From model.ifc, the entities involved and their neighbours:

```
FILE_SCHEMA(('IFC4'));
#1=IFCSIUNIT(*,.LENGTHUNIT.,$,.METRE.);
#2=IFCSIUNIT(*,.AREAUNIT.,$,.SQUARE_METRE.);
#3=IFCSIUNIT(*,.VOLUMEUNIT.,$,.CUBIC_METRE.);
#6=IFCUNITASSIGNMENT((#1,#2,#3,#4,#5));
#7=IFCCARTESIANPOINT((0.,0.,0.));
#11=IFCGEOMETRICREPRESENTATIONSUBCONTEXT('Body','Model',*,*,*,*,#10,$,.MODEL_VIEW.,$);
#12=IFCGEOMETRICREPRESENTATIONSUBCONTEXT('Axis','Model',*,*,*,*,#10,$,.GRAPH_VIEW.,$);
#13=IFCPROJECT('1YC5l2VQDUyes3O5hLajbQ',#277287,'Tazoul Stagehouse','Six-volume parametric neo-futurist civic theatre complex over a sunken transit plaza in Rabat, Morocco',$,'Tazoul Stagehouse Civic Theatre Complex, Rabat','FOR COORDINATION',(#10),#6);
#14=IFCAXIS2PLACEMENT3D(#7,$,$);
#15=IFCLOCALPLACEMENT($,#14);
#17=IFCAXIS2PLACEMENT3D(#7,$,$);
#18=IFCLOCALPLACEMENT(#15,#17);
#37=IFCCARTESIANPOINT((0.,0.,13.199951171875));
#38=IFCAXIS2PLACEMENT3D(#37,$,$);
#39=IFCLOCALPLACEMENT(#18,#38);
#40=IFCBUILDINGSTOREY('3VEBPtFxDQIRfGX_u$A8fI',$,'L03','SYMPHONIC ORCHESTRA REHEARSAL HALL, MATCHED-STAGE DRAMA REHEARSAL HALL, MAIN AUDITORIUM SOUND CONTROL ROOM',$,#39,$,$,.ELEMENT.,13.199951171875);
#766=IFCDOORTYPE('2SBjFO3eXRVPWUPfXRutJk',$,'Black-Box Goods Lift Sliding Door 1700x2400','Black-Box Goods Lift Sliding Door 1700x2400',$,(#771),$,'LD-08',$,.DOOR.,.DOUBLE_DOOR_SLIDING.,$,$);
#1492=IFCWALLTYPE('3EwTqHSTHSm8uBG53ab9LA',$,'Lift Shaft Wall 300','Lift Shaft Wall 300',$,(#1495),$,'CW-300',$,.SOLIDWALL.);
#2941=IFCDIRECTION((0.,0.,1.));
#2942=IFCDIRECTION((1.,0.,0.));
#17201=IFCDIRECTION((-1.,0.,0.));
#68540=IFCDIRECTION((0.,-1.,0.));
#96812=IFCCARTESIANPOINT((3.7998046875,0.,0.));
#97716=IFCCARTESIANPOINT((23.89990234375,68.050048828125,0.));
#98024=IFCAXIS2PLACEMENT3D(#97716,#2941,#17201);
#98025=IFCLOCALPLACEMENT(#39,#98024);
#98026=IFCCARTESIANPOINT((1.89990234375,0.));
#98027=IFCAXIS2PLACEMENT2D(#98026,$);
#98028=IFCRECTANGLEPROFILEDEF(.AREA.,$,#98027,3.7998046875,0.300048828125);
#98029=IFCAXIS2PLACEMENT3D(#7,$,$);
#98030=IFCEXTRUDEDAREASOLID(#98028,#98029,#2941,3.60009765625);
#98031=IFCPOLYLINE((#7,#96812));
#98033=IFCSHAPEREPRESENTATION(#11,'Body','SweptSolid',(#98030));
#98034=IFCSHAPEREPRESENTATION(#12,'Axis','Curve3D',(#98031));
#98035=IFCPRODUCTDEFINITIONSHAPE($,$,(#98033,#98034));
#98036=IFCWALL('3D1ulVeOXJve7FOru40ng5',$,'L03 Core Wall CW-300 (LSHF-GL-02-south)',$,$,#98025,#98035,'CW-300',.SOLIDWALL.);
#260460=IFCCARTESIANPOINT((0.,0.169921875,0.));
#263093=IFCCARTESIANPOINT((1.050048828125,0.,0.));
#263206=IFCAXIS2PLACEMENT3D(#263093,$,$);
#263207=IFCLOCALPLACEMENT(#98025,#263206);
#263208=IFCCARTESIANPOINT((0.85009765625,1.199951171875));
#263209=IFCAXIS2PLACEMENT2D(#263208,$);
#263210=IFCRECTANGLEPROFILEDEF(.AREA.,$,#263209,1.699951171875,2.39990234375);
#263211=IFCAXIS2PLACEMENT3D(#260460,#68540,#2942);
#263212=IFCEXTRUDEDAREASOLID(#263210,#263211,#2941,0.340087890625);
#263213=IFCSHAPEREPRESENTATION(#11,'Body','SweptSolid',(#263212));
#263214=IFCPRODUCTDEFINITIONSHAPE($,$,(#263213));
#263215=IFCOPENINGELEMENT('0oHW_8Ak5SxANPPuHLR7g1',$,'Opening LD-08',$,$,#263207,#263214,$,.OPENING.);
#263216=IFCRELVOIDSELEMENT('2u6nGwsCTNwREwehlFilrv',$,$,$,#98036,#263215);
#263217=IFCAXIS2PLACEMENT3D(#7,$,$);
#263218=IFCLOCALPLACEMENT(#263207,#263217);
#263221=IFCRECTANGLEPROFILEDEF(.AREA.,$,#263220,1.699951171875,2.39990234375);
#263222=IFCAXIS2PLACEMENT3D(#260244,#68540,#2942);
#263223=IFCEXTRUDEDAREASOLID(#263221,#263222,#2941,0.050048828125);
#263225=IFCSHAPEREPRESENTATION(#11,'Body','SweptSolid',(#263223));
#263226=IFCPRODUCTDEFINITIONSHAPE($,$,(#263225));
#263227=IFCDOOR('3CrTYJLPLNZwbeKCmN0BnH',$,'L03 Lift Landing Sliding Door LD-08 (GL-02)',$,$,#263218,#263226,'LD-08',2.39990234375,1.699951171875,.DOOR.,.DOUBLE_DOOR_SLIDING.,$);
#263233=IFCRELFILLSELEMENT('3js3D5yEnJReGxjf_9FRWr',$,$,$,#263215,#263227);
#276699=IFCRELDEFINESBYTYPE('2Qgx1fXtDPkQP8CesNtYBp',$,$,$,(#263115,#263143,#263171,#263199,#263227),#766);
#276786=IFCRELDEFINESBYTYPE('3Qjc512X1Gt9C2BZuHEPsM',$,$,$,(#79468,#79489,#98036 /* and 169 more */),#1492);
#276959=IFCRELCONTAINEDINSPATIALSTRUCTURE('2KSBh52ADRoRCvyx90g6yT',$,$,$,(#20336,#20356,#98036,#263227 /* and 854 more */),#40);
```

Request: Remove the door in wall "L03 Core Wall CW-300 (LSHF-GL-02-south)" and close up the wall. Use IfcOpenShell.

```python
import ifcopenshell
import ifcopenshell.api.feature
import ifcopenshell.api.root
import ifcopenshell.geom
import ifcopenshell.util.shape

model = ifcopenshell.open("model.ifc")
settings = ifcopenshell.geom.settings()


def volume(element):
    """Net volume in cubic metres, openings subtracted."""
    shape = ifcopenshell.geom.create_shape(settings, element)
    return ifcopenshell.util.shape.get_volume(shape.geometry)


door = model.by_id(263227)
opening = door.FillsVoids[0].RelatingOpeningElement
wall = opening.VoidsElements[0].RelatingBuildingElement
before = volume(wall)

ifcopenshell.api.root.remove_product(model, product=door)
ifcopenshell.api.feature.remove_feature(model, feature=opening)

after = volume(wall)

print(f"wall volume {before:.3f} -> {after:.3f} m3")

model.write("model_updated.ifc")
```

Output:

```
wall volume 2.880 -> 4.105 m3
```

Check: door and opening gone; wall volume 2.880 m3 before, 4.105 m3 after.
